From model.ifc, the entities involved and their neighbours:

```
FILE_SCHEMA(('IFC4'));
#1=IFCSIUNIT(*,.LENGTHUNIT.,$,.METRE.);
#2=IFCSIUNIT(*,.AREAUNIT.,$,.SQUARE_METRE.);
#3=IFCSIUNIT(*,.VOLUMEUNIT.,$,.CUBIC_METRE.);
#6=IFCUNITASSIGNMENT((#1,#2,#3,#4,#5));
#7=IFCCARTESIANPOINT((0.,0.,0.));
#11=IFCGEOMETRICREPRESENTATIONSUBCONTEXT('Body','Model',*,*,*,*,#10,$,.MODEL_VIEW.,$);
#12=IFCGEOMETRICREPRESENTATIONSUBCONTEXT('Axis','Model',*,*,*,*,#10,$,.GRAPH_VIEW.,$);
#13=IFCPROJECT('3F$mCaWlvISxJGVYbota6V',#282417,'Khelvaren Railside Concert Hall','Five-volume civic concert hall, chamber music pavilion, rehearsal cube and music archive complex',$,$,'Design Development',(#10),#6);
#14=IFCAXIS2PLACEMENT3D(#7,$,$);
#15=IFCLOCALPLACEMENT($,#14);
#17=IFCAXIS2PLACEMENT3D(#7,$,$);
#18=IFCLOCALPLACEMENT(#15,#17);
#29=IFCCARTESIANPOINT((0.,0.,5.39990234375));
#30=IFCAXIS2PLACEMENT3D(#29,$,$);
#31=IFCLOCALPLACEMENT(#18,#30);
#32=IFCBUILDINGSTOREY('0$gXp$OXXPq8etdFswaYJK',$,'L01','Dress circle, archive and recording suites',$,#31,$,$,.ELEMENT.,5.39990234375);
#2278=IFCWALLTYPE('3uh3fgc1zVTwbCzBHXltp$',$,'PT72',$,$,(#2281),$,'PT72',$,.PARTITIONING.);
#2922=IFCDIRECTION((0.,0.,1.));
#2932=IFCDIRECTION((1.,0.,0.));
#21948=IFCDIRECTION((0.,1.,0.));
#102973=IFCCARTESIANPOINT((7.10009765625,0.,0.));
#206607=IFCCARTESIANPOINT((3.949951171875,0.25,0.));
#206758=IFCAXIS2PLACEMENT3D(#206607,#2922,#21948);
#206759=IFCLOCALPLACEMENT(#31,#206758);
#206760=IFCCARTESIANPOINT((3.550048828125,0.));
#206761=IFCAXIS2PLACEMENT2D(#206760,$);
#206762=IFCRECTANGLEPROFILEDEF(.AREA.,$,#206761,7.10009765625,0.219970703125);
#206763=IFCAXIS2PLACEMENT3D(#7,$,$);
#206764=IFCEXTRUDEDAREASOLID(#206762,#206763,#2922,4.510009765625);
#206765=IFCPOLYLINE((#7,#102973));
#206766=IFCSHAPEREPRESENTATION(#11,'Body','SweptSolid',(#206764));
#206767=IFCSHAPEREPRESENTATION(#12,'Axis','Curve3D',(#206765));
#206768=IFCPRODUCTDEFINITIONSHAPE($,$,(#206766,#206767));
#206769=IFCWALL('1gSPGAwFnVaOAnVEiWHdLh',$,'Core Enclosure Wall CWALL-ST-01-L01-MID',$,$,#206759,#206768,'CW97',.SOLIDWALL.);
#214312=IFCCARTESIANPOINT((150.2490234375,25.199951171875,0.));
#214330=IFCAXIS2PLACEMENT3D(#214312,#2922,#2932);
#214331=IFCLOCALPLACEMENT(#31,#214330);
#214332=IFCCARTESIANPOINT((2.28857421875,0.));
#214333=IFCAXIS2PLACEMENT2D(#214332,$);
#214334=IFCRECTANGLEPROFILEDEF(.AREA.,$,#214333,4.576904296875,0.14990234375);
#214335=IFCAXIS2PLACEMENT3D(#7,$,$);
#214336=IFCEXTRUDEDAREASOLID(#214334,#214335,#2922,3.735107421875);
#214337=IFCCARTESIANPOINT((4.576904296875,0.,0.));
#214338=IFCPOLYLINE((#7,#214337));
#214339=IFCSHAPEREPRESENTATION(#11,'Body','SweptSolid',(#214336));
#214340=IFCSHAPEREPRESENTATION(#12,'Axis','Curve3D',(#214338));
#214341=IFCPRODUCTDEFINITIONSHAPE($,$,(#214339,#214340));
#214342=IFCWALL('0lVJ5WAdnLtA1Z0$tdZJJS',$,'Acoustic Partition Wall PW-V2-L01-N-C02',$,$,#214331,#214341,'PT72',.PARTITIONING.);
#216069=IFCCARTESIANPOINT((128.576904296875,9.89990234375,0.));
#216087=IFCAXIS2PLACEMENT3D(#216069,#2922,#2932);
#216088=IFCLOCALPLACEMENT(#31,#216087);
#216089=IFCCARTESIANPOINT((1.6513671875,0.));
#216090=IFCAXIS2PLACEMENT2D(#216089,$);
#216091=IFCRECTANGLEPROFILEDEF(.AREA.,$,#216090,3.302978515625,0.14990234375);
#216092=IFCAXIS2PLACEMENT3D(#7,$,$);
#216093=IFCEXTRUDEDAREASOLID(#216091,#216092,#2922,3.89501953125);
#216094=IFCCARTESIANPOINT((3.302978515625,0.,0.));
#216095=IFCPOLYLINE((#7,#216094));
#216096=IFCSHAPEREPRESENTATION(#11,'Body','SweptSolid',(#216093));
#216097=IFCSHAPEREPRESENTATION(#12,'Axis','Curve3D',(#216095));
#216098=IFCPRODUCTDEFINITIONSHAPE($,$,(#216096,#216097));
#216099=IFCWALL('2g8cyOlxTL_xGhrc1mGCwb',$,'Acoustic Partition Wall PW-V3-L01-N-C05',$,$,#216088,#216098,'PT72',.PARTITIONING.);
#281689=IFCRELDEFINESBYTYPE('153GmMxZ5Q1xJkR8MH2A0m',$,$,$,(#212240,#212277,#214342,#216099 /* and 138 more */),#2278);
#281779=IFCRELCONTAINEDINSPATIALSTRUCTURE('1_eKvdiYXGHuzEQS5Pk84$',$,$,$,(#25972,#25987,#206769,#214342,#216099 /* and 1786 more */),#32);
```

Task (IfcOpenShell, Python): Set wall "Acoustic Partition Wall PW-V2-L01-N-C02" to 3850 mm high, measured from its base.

```python
import ifcopenshell
import ifcopenshell.geom
import ifcopenshell.util.representation
import ifcopenshell.util.shape
import ifcopenshell.util.unit

model = ifcopenshell.open("model.ifc")
unit_scale = ifcopenshell.util.unit.calculate_unit_scale(model)
settings = ifcopenshell.geom.settings()


def volume(element):
    """Net volume in cubic metres, openings subtracted."""
    shape = ifcopenshell.geom.create_shape(settings, element)
    return ifcopenshell.util.shape.get_volume(shape.geometry)


wall = model.by_id(214342)
before = volume(wall)

body = ifcopenshell.util.representation.get_representation(wall, "Model", "Body")
solid = body.Items[0]
old_height = solid.Depth
solid.Depth = 3.85 / unit_scale
after = volume(wall)

print(f"height {old_height:g} -> {solid.Depth:g}, volume {before:.3f} -> {after:.3f} m3")

model.write("model_v2.ifc")
```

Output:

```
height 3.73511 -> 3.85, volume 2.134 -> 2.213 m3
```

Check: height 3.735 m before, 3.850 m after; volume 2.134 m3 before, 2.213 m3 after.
